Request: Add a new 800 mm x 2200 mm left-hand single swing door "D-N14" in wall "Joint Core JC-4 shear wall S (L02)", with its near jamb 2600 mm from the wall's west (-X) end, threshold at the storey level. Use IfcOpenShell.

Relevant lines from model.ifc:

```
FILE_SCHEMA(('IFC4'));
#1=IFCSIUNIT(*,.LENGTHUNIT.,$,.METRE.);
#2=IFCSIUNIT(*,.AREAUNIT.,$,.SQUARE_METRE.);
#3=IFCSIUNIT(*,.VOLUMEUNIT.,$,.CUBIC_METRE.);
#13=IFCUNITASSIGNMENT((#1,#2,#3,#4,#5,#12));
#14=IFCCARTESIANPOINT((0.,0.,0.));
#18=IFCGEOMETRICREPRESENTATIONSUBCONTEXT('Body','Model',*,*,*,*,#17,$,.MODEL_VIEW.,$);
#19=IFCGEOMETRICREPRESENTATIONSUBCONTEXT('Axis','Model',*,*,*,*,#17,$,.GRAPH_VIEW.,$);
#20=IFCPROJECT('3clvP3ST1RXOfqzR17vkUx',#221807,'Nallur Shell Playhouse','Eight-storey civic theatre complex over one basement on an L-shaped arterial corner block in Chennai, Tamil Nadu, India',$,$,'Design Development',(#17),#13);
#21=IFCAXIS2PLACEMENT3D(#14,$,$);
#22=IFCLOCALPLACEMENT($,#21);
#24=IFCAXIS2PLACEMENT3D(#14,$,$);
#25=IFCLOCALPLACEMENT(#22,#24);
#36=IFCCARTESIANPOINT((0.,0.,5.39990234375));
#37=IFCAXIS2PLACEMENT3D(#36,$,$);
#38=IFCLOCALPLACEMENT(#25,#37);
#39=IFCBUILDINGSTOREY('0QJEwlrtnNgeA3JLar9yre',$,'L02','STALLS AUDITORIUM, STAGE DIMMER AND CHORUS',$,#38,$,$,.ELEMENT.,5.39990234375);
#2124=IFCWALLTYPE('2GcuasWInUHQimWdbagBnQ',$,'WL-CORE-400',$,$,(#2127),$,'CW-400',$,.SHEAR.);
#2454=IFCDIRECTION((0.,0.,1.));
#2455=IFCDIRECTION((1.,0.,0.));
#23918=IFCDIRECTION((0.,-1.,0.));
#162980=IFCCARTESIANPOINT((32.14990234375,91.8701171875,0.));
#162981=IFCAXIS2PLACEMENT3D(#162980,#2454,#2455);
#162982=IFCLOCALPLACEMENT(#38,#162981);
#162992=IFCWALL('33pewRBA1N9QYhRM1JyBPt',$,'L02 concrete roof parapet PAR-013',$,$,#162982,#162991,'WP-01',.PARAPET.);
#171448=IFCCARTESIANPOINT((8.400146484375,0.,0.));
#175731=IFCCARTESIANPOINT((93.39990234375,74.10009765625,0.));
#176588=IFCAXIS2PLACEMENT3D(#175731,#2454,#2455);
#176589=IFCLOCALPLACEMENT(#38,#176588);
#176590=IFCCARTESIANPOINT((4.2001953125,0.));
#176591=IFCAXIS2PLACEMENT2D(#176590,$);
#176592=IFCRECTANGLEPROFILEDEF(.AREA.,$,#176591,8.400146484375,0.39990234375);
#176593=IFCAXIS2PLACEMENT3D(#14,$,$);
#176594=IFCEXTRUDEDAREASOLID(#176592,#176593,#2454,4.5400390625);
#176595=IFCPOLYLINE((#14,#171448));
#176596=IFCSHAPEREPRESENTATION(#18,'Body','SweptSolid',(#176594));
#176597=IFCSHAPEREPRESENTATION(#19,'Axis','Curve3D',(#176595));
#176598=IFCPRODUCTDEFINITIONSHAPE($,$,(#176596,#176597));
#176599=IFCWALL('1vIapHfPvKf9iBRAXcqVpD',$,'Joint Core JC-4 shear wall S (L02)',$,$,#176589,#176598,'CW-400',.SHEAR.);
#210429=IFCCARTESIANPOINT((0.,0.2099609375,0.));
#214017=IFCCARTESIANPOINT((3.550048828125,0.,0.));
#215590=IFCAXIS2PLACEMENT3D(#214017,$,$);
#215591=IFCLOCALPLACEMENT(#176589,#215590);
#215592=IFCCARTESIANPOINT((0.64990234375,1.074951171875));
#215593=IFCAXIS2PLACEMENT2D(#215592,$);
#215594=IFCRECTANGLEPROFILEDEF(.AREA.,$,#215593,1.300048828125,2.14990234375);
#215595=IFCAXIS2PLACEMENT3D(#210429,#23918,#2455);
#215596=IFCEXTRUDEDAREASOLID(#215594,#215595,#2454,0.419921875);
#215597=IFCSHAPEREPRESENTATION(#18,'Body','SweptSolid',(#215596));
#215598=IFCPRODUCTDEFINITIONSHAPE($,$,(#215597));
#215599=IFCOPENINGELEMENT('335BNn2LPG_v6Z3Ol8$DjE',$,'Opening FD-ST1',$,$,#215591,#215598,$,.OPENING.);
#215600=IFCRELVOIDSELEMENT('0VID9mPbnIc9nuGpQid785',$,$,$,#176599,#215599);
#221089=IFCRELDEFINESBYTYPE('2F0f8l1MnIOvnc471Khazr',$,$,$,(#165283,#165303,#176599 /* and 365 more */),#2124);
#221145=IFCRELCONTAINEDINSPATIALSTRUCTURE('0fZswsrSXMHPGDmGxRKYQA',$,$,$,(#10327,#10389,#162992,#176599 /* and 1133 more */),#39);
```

```python
import numpy as np
import ifcopenshell
import ifcopenshell.api.feature
import ifcopenshell.api.geometry
import ifcopenshell.api.root
import ifcopenshell.api.spatial
import ifcopenshell.geom
import ifcopenshell.util.element
import ifcopenshell.util.placement
import ifcopenshell.util.representation
import ifcopenshell.util.shape
import ifcopenshell.util.unit

model = ifcopenshell.open("model.ifc")
unit_scale = ifcopenshell.util.unit.calculate_unit_scale(model)
settings = ifcopenshell.geom.settings()


def volume(element):
    """Net volume in cubic metres, openings subtracted."""
    shape = ifcopenshell.geom.create_shape(settings, element)
    return ifcopenshell.util.shape.get_volume(shape.geometry)


wall = model.by_guid("1vIapHfPvKf9iBRAXcqVpD")
storey = ifcopenshell.util.element.get_container(wall, ifc_class="IfcBuildingStorey")
context = ifcopenshell.util.representation.get_context(model, "Model", "Body", "MODEL_VIEW")
before = volume(wall)

width, height, from_end, sill = 0.8, 2.2, 2.6, 0.0  # metres

# The wall runs along its own X axis, and the end named is its -X end.
wall_shape = ifcopenshell.geom.create_shape(settings, wall)
x, y, z = ifcopenshell.util.shape.get_vertices(wall_shape.geometry).T
start = x.min() + from_end
face, thickness = float(y.min()), float(y.max() - y.min())
wall_matrix = ifcopenshell.util.placement.get_local_placement(wall.ObjectPlacement)
level = ifcopenshell.util.placement.get_local_placement(storey.ObjectPlacement)[2, 3]


def in_wall(x, y):
    """Placement at x, y metres in the wall's axes, at sill height."""
    matrix = wall_matrix.copy()
    matrix[:, 3] = wall_matrix @ np.array([x / unit_scale, y / unit_scale, 0.0, 1.0])
    matrix[2, 3] = level + sill / unit_scale
    return matrix


# Opening: a box that overshoots both wall faces by 50 mm.
opening = ifcopenshell.api.root.create_entity(model, ifc_class="IfcOpeningElement", predefined_type="OPENING")
box = ifcopenshell.api.geometry.add_wall_representation(
    model, context=context, length=width, height=height, thickness=thickness + 0.1
)
ifcopenshell.api.geometry.assign_representation(model, product=opening, representation=box)
ifcopenshell.api.geometry.edit_object_placement(model, product=opening, matrix=in_wall(start, face - 0.05), is_si=False)
ifcopenshell.api.feature.add_feature(model, feature=opening, element=wall)

door = ifcopenshell.api.root.create_entity(model, ifc_class="IfcDoor", name="D-N14", predefined_type="DOOR")
door.OverallWidth, door.OverallHeight = width / unit_scale, height / unit_scale
door.OperationType = "SINGLE_SWING_LEFT"
body = ifcopenshell.api.geometry.add_door_representation(
    model,
    context=context,
    overall_width=door.OverallWidth,
    overall_height=door.OverallHeight,
    operation_type="SINGLE_SWING_LEFT",
    lining_properties={"LiningDepth": thickness / unit_scale, "ThresholdDepth": thickness / unit_scale},
)
ifcopenshell.api.geometry.assign_representation(model, product=door, representation=body)
ifcopenshell.api.spatial.assign_container(model, products=[door], relating_structure=storey)
ifcopenshell.api.feature.add_filling(model, opening=opening, element=door)

# The lining spans the wall, so the door starts at the wall face.
ifcopenshell.api.geometry.edit_object_placement(model, product=door, matrix=in_wall(start, face), is_si=False)

after = volume(wall)

print(f"wall volume {before:.3f} -> {after:.3f} m3")

model.write("model_v2.ifc")
```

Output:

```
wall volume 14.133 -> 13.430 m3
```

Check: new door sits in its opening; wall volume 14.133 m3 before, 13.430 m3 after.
